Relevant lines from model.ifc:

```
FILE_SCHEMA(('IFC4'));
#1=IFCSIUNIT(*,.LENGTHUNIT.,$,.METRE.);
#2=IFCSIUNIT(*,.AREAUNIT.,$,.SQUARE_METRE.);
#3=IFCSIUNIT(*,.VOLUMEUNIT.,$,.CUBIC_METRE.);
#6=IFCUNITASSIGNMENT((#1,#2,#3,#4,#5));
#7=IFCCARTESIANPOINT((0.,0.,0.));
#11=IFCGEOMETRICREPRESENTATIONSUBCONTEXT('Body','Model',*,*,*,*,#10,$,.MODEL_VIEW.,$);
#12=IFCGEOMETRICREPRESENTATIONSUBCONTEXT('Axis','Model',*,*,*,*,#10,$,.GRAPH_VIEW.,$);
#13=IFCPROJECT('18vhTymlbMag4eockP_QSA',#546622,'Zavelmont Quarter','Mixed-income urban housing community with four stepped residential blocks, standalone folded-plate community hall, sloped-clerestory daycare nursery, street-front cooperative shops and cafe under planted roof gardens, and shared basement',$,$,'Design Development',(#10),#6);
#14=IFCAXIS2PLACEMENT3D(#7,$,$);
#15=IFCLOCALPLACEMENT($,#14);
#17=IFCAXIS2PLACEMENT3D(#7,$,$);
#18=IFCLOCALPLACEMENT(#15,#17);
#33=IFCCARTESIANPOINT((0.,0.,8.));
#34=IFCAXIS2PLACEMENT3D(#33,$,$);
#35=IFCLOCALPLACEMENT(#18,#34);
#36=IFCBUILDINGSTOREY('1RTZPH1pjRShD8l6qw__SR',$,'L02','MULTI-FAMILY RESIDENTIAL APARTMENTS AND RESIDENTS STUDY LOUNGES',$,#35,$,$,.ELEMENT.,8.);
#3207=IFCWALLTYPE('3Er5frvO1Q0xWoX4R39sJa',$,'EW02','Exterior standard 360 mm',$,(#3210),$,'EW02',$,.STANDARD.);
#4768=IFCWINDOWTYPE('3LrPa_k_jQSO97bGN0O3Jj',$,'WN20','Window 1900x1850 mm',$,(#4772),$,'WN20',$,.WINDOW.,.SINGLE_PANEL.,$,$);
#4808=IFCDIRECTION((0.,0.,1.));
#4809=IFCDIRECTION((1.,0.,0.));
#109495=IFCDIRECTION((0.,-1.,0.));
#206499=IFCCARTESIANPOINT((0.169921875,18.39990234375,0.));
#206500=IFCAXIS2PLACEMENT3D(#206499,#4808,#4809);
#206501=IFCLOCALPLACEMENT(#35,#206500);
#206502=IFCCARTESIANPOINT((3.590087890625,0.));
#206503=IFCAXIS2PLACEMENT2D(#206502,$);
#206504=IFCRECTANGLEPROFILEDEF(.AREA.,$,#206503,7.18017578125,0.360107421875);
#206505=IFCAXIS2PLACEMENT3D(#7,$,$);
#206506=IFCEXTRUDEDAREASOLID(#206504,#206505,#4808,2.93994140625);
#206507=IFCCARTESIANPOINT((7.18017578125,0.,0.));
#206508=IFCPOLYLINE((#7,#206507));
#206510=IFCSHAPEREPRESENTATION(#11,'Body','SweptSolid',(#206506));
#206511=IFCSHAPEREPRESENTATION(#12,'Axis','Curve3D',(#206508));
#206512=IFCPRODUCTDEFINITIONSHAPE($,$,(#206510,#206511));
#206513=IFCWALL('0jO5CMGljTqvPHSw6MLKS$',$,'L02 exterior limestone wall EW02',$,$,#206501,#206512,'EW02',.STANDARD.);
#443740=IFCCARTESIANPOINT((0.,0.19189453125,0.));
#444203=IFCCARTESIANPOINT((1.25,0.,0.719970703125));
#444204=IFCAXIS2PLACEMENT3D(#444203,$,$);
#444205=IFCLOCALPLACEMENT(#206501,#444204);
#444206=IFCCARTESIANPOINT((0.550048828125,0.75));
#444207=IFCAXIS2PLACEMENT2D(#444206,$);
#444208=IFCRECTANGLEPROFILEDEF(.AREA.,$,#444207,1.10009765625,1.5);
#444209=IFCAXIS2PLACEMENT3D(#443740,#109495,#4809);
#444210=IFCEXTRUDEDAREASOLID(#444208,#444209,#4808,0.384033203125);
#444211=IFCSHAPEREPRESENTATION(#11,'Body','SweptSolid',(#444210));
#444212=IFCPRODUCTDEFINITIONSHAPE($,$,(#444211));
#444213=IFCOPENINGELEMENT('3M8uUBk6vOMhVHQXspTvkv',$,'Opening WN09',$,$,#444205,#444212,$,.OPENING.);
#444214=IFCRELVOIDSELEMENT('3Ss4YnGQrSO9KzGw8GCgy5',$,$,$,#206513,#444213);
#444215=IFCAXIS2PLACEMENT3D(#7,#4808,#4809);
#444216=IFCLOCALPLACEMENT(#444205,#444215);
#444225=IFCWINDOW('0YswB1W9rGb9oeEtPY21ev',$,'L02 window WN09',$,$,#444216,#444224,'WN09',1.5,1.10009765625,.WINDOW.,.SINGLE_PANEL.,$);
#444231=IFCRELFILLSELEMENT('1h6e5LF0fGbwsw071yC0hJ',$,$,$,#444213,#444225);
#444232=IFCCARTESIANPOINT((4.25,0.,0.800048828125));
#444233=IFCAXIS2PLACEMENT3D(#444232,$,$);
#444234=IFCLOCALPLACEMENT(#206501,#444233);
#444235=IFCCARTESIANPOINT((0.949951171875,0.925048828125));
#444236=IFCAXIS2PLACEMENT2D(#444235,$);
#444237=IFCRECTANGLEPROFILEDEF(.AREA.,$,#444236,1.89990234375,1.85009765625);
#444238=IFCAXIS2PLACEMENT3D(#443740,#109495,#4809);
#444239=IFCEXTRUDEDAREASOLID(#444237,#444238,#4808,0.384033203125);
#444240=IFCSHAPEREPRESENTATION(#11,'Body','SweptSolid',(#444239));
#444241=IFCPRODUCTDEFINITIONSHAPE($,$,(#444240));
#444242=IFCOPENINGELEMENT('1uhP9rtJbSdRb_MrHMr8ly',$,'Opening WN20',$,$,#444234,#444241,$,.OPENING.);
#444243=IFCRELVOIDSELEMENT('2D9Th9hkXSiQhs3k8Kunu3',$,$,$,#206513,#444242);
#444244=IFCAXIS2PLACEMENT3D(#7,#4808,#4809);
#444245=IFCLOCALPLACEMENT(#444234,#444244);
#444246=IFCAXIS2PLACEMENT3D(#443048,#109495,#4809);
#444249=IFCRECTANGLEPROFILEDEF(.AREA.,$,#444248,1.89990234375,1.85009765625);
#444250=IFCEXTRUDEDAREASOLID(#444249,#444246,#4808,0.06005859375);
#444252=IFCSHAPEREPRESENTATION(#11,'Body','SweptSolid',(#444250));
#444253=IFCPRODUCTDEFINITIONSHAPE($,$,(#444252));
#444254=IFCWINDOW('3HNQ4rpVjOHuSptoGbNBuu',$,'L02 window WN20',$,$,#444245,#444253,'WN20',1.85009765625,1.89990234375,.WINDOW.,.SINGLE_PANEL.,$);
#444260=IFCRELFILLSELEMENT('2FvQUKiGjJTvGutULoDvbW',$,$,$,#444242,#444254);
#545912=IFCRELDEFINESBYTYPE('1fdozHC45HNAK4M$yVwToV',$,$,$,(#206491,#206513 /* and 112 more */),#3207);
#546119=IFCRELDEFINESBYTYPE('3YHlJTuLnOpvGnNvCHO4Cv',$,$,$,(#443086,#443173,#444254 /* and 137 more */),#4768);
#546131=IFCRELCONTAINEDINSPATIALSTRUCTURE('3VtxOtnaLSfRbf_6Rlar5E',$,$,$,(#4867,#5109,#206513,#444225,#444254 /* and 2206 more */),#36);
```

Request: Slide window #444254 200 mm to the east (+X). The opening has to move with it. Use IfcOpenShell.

```python
import ifcopenshell
import ifcopenshell.api.geometry
import ifcopenshell.util.placement
import ifcopenshell.util.unit

model = ifcopenshell.open("model.ifc")
unit_scale = ifcopenshell.util.unit.calculate_unit_scale(model)

window = model.by_guid("3HNQ4rpVjOHuSptoGbNBuu")
opening = window.FillsVoids[0].RelatingOpeningElement
wall = opening.VoidsElements[0].RelatingBuildingElement

wall_matrix = ifcopenshell.util.placement.get_local_placement(wall.ObjectPlacement)
shift = wall_matrix[:3, 0] * 0.2 / unit_scale
before = ifcopenshell.util.placement.get_local_placement(window.ObjectPlacement)[:3, 3].copy()

# The window is placed relative to its opening, so it follows when the opening moves.
matrix = ifcopenshell.util.placement.get_local_placement(opening.ObjectPlacement)
matrix[:3, 3] += shift
ifcopenshell.api.geometry.edit_object_placement(
    model, product=opening, matrix=matrix, is_si=False, should_transform_children=True
)

after = ifcopenshell.util.placement.get_local_placement(window.ObjectPlacement)[:3, 3]
print("window moved by", (after - before).round(3) + 0.0)

model.write("model_updated.ifc")
```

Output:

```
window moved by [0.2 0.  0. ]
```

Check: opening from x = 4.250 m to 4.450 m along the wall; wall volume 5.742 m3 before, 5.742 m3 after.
